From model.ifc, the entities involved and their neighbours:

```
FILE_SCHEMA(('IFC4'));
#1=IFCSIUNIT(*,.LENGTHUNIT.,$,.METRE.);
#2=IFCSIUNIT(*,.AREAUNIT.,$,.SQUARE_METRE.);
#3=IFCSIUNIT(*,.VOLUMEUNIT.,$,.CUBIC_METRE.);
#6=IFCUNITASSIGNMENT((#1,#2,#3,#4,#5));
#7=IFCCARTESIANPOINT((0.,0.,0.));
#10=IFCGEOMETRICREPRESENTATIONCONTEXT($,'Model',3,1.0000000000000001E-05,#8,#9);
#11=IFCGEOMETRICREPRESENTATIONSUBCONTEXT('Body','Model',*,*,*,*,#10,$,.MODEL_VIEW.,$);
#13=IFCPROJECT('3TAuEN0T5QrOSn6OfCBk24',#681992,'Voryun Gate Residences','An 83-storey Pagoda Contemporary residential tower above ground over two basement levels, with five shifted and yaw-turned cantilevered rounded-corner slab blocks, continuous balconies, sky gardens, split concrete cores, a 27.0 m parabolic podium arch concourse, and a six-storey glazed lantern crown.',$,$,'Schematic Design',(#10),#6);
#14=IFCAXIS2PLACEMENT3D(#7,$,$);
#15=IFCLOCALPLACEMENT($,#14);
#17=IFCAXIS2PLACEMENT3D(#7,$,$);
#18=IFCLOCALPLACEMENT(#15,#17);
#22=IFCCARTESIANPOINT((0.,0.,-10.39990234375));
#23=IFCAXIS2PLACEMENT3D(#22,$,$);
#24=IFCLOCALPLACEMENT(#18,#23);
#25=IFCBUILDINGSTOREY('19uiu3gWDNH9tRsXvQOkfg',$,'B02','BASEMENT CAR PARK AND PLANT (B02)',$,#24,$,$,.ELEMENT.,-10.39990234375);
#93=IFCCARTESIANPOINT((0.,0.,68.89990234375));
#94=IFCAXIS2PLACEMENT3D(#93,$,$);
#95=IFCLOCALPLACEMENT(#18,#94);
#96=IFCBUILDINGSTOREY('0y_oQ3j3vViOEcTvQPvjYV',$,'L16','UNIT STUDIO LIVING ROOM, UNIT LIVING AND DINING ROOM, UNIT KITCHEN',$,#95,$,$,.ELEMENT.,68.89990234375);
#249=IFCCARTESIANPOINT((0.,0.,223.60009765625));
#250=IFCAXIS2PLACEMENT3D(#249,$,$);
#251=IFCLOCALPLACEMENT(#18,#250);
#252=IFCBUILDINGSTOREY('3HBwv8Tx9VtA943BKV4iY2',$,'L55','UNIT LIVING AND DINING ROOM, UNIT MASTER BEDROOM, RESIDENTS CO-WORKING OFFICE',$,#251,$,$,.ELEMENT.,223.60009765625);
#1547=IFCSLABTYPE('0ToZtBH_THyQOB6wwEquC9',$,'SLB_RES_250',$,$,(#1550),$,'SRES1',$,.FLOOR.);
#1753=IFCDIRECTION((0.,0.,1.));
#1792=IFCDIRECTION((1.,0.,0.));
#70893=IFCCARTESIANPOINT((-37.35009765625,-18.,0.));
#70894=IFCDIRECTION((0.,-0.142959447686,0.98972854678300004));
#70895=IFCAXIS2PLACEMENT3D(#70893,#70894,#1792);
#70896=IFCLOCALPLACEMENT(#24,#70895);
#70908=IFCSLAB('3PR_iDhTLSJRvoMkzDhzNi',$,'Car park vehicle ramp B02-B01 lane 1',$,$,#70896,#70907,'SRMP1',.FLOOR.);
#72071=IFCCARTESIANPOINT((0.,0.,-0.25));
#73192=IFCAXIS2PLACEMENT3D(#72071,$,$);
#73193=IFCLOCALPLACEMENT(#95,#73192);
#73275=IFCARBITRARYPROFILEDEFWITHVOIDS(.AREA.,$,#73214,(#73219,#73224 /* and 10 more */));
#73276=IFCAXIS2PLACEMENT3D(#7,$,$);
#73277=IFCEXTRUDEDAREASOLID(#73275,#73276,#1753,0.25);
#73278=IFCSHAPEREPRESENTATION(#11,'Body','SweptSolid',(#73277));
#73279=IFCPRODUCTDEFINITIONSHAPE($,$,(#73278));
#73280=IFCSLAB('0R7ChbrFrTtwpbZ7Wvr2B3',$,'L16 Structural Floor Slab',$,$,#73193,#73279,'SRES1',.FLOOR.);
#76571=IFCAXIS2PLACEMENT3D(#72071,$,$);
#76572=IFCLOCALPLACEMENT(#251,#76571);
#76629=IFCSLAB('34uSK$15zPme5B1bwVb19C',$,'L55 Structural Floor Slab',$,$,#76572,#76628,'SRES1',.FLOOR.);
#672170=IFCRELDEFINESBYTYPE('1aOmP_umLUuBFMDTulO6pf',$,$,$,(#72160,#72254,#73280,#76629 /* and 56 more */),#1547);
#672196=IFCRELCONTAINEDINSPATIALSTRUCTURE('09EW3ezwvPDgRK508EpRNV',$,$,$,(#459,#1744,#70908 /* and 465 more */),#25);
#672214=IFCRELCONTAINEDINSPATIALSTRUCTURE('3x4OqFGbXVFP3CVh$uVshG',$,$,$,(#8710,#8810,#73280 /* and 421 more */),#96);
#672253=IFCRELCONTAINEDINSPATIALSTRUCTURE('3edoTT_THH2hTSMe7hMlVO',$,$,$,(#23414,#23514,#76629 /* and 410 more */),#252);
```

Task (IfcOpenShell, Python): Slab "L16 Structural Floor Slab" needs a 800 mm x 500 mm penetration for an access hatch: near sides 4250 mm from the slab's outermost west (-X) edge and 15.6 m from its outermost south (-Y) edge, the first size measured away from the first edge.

```python
import numpy as np
import ifcopenshell
import ifcopenshell.api.feature
import ifcopenshell.api.geometry
import ifcopenshell.api.root
import ifcopenshell.geom
import ifcopenshell.util.placement
import ifcopenshell.util.representation
import ifcopenshell.util.shape
import ifcopenshell.util.unit

model = ifcopenshell.open("model.ifc")
unit_scale = ifcopenshell.util.unit.calculate_unit_scale(model)
settings = ifcopenshell.geom.settings()


def volume(element):
    """Net volume in cubic metres, openings subtracted."""
    shape = ifcopenshell.geom.create_shape(settings, element)
    return ifcopenshell.util.shape.get_volume(shape.geometry)


slab = model.by_guid("0R7ChbrFrTtwpbZ7Wvr2B3")
before = volume(slab)

# Extent in the slab's own axes, in metres. The edges named are its -X and -Y sides.
slab_shape = ifcopenshell.geom.create_shape(settings, slab)
vertices = ifcopenshell.util.shape.get_vertices(slab_shape.geometry)
x_min, y_min, bottom = vertices.min(axis=0)
top = vertices[:, 2].max()

opening = ifcopenshell.api.root.create_entity(model, ifc_class="IfcOpeningElement", name="Access hatch opening", predefined_type="OPENING")
context = ifcopenshell.util.representation.get_context(model, "Model", "Body", "MODEL_VIEW")
width, depth = 0.8, 0.5
outline = [(0.0, 0.0), (width, 0.0), (width, depth), (0.0, depth), (0.0, 0.0)]
# Overshoot both faces by 50 mm so the cut is clean.
shape = ifcopenshell.api.geometry.add_slab_representation(
    model, context=context, depth=top - bottom + 0.1, polyline=outline
)
ifcopenshell.api.geometry.assign_representation(model, product=opening, representation=shape)

matrix = ifcopenshell.util.placement.get_local_placement(slab.ObjectPlacement)
matrix[:, 3] = matrix @ np.append(np.array([x_min + 4.25, y_min + 15.6, bottom - 0.05]) / unit_scale, 1.0)
ifcopenshell.api.geometry.edit_object_placement(model, product=opening, matrix=matrix, is_si=False)
ifcopenshell.api.feature.add_feature(model, feature=opening, element=slab)

after = volume(slab)

print(f"slab volume {before:.3f} -> {after:.3f} m3")

model.write("model-out.ifc")
```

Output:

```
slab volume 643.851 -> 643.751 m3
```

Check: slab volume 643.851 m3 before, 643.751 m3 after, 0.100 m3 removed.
